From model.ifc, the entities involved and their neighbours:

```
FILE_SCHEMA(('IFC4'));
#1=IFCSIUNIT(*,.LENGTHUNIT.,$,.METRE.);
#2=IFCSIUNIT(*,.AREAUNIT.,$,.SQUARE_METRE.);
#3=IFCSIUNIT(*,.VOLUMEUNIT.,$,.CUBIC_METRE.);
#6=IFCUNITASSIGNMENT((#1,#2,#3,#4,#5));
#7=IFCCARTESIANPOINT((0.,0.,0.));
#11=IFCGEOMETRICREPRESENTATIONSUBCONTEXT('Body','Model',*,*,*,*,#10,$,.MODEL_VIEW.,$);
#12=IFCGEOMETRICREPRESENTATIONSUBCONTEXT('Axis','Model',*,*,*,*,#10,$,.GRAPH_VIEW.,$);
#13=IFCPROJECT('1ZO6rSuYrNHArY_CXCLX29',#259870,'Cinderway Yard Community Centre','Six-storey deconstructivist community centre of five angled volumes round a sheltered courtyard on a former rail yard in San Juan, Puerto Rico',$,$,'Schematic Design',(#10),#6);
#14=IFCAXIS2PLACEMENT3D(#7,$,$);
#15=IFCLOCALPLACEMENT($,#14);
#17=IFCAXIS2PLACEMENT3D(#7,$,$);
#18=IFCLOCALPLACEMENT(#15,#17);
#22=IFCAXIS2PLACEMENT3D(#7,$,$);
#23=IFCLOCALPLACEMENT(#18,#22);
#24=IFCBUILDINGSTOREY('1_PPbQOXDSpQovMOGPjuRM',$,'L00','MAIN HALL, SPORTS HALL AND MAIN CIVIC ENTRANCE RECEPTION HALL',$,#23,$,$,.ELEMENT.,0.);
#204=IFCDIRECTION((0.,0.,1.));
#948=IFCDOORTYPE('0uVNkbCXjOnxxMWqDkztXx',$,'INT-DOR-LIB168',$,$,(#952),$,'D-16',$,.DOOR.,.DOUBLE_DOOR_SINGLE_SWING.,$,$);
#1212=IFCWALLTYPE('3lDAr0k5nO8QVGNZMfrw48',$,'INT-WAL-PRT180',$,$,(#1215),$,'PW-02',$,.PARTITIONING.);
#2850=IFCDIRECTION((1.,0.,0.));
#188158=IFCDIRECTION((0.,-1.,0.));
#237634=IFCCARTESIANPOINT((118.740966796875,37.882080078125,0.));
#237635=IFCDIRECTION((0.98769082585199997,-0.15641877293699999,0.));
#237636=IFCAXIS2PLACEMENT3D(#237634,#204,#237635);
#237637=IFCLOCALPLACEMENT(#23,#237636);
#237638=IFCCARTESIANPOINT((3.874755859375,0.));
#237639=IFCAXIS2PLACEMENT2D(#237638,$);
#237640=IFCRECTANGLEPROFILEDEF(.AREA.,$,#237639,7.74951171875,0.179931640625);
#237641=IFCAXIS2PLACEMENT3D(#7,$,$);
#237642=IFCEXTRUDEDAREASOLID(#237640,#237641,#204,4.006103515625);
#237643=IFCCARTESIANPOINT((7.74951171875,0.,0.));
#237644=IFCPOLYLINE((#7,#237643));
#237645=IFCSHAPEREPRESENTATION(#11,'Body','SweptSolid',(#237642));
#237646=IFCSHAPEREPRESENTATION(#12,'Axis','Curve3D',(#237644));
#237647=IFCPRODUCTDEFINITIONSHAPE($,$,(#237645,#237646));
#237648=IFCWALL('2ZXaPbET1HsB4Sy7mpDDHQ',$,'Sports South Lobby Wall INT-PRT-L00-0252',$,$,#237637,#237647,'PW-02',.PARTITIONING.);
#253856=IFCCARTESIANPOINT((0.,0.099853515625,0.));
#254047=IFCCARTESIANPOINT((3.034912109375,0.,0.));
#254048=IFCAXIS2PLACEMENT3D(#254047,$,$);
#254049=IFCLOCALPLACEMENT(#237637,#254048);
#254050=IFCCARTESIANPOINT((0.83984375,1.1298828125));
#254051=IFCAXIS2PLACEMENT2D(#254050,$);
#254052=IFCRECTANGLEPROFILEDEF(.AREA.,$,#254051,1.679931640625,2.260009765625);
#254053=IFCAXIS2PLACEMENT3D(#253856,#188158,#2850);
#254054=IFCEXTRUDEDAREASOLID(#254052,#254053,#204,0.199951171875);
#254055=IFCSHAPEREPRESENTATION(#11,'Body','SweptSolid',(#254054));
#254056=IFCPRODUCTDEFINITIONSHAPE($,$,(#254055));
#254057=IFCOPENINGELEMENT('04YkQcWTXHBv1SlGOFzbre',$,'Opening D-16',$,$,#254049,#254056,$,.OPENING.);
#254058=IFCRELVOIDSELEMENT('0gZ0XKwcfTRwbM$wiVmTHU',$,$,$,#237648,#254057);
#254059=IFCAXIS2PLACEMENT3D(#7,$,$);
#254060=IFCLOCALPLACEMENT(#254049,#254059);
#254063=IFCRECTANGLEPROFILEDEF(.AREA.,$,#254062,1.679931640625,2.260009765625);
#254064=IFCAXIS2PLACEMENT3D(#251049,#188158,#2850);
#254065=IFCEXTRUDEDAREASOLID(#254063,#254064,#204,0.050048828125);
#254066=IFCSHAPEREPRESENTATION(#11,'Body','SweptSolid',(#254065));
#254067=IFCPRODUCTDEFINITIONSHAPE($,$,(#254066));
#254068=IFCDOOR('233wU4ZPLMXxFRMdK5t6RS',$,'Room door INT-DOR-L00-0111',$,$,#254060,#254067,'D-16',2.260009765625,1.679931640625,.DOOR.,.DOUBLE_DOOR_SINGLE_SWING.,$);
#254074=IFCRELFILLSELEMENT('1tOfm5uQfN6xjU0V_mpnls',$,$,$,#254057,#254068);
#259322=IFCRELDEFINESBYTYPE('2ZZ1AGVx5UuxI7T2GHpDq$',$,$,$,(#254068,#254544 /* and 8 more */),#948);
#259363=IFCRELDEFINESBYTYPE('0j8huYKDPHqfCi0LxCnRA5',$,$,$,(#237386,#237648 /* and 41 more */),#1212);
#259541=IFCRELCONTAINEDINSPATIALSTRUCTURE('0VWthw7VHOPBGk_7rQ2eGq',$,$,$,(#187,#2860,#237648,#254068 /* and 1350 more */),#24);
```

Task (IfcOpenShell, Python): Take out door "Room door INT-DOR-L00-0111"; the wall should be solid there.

```python
import ifcopenshell
import ifcopenshell.api.feature
import ifcopenshell.api.root
import ifcopenshell.geom
import ifcopenshell.util.shape

model = ifcopenshell.open("model.ifc")
settings = ifcopenshell.geom.settings()


def volume(element):
    """Net volume in cubic metres, openings subtracted."""
    shape = ifcopenshell.geom.create_shape(settings, element)
    return ifcopenshell.util.shape.get_volume(shape.geometry)


door = model.by_guid("233wU4ZPLMXxFRMdK5t6RS")
opening = door.FillsVoids[0].RelatingOpeningElement
wall = opening.VoidsElements[0].RelatingBuildingElement
before = volume(wall)

ifcopenshell.api.root.remove_product(model, product=door)
ifcopenshell.api.feature.remove_feature(model, feature=opening)

after = volume(wall)

print(f"wall volume {before:.3f} -> {after:.3f} m3")

model.write("model_edited.ifc")
```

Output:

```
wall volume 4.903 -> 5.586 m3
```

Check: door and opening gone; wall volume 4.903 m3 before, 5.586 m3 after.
